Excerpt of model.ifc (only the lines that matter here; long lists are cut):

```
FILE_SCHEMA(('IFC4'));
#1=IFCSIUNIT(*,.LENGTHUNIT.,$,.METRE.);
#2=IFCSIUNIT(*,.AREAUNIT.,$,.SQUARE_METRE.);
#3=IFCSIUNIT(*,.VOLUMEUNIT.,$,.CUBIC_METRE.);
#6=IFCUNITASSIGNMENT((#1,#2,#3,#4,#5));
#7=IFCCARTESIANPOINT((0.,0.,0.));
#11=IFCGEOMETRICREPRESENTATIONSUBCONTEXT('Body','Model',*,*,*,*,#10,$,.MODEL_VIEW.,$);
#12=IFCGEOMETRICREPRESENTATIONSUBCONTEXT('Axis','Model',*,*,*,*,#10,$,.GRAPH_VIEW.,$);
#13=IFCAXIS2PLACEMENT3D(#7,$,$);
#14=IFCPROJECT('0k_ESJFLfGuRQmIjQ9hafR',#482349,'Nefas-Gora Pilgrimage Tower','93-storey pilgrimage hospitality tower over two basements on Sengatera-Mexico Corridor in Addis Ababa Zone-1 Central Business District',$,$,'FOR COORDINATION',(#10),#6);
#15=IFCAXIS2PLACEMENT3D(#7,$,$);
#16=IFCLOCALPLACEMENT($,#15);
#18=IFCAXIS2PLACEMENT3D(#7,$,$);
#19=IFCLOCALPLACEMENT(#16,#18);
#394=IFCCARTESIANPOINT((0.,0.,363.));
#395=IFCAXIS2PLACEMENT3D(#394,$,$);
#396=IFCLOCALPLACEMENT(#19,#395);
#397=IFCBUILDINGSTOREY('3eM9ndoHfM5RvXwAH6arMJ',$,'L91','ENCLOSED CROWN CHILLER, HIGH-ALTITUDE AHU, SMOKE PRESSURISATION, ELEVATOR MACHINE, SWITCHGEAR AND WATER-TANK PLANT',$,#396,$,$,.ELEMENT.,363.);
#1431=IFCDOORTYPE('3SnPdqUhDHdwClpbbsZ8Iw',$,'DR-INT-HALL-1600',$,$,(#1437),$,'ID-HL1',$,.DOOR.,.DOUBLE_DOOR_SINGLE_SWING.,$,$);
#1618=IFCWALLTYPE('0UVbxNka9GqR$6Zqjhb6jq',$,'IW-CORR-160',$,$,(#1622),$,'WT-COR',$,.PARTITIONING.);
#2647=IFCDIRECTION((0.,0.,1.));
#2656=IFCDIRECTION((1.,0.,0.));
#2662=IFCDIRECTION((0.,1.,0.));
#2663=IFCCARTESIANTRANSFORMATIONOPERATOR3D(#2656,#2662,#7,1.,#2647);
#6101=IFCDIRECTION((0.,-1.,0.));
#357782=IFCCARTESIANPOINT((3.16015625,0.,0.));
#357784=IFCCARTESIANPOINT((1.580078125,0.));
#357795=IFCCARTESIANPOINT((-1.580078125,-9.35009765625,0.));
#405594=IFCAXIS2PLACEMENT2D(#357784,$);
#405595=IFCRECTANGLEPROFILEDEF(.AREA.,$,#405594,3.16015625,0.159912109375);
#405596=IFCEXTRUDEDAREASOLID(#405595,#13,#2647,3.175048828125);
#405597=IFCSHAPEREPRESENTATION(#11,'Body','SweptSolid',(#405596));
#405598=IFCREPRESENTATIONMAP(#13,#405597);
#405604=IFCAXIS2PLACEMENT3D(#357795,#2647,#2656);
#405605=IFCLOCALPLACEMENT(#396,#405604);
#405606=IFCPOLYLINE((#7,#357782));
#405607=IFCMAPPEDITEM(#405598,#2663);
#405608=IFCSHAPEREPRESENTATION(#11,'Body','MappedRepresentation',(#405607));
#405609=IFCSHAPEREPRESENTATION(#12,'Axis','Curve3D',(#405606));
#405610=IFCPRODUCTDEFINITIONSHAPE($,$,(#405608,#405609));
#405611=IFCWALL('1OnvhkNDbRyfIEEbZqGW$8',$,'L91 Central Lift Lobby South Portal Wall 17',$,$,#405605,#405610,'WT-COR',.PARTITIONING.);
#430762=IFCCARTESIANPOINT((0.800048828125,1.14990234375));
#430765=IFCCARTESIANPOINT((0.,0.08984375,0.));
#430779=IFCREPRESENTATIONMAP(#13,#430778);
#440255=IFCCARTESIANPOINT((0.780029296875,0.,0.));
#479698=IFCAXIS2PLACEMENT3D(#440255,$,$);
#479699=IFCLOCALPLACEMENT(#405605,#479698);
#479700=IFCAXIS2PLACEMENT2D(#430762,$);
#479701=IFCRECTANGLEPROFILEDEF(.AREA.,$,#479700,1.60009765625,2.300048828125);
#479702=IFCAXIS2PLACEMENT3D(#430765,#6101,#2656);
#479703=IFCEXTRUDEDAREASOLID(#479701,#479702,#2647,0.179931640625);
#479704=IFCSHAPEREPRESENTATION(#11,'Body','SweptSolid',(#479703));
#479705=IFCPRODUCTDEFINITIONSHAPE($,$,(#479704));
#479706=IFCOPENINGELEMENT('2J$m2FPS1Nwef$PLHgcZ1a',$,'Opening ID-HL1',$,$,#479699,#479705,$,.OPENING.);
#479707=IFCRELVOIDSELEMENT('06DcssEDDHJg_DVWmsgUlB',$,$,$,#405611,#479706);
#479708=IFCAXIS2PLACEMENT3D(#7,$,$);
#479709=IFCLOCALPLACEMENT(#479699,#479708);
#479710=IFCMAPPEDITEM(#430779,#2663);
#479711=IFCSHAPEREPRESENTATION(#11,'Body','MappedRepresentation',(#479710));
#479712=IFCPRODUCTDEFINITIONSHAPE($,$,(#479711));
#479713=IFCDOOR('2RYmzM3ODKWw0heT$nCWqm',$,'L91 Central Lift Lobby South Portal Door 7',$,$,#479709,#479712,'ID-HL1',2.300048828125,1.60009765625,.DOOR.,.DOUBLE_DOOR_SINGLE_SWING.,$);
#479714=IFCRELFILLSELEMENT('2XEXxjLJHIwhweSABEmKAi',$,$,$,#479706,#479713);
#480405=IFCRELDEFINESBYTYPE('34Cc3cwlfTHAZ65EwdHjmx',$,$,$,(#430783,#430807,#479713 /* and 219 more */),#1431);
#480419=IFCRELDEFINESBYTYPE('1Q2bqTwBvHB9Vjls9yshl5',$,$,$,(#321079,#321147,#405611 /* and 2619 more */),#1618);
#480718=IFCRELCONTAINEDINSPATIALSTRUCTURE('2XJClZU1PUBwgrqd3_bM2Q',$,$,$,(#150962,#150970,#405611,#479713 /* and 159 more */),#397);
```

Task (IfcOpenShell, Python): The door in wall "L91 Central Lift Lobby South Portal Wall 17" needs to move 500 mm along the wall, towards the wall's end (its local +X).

```python
import ifcopenshell
import ifcopenshell.api.geometry
import ifcopenshell.util.placement
import ifcopenshell.util.unit

model = ifcopenshell.open("model.ifc")
unit_scale = ifcopenshell.util.unit.calculate_unit_scale(model)

door = model.by_guid("2RYmzM3ODKWw0heT$nCWqm")
opening = door.FillsVoids[0].RelatingOpeningElement
wall = opening.VoidsElements[0].RelatingBuildingElement

wall_matrix = ifcopenshell.util.placement.get_local_placement(wall.ObjectPlacement)
shift = wall_matrix[:3, 0] * 0.5 / unit_scale
before = ifcopenshell.util.placement.get_local_placement(door.ObjectPlacement)[:3, 3].copy()

# The door is placed relative to its opening, so it follows when the opening moves.
matrix = ifcopenshell.util.placement.get_local_placement(opening.ObjectPlacement)
matrix[:3, 3] += shift
ifcopenshell.api.geometry.edit_object_placement(
    model, product=opening, matrix=matrix, is_si=False, should_transform_children=True
)

after = ifcopenshell.util.placement.get_local_placement(door.ObjectPlacement)[:3, 3]
print("door moved by", (after - before).round(3) + 0.0)

model.write("model_v2.ifc")
```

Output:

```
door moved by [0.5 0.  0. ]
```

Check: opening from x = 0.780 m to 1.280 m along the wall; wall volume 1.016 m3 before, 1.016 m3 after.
